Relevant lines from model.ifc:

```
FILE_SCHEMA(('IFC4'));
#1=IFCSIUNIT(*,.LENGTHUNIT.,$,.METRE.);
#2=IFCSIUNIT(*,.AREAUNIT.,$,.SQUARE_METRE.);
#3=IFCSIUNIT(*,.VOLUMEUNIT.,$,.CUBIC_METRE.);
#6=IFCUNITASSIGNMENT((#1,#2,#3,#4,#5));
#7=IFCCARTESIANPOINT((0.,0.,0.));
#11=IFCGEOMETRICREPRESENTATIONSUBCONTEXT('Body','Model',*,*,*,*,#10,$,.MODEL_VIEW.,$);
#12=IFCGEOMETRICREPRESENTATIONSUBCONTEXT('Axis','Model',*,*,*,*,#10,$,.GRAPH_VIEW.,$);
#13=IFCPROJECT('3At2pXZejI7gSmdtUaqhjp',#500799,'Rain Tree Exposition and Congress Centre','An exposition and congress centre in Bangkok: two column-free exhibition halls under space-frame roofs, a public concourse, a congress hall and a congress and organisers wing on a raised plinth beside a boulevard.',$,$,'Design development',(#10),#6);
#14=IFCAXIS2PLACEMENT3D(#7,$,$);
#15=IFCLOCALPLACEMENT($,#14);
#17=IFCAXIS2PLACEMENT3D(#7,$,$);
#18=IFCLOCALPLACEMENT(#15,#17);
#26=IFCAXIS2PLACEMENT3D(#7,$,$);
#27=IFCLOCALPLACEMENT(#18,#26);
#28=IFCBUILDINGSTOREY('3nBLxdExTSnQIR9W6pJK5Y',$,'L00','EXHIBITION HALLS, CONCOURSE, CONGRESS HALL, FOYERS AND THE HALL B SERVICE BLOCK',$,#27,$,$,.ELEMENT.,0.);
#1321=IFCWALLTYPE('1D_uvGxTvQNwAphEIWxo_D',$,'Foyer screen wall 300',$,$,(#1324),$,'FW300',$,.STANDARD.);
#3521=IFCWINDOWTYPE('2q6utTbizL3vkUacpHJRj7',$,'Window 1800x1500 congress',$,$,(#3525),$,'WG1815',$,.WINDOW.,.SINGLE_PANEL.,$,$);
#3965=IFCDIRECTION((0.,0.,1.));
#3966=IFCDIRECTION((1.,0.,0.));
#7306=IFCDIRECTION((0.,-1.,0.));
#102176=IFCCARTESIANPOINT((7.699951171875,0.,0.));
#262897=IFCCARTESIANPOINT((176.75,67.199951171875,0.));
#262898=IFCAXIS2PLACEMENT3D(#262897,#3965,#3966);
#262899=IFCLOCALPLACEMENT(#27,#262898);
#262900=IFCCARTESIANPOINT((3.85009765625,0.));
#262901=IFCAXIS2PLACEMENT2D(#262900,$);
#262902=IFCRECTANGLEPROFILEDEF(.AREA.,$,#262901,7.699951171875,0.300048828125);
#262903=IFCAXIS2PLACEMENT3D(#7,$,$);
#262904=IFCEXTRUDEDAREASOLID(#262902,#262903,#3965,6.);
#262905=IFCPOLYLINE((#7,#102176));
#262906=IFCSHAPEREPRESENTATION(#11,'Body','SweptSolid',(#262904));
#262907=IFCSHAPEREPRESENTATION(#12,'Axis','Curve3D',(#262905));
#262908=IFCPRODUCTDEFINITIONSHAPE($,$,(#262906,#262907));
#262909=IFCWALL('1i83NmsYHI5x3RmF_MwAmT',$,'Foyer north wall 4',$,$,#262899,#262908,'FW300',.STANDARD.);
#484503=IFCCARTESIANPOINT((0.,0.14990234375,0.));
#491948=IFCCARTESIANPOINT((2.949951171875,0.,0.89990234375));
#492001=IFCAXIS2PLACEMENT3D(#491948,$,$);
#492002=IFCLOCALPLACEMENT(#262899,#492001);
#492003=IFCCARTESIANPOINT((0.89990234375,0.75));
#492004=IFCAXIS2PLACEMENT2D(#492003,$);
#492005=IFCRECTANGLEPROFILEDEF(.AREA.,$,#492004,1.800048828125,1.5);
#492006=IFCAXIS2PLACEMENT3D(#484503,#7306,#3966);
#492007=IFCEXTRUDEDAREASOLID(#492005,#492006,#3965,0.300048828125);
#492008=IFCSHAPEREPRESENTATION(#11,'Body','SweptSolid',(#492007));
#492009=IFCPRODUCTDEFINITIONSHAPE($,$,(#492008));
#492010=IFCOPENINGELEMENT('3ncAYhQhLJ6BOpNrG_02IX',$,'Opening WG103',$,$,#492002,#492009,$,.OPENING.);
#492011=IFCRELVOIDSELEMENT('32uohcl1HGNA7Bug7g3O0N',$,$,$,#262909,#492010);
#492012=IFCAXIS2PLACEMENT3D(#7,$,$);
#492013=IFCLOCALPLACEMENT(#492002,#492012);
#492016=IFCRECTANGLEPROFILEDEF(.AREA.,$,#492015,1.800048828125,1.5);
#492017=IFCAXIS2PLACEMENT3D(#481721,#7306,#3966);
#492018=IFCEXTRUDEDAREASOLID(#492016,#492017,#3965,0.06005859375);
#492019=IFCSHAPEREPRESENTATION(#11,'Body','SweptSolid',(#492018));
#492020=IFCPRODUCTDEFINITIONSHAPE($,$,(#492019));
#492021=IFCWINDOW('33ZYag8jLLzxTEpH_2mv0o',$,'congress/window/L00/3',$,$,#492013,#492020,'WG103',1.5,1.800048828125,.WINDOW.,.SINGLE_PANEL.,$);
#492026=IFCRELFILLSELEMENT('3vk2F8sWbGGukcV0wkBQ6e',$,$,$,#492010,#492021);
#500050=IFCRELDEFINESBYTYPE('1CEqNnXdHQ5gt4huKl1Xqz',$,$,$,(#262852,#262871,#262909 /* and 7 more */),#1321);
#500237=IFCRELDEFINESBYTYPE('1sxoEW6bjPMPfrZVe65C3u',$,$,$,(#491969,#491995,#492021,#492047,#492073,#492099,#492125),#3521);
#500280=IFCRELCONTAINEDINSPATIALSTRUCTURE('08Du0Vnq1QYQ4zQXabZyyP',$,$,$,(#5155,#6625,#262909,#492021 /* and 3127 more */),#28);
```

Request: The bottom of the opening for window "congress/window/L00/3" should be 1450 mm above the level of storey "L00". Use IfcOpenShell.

```python
import numpy as np
import ifcopenshell
import ifcopenshell.api.geometry
import ifcopenshell.geom
import ifcopenshell.util.element
import ifcopenshell.util.placement
import ifcopenshell.util.shape
import ifcopenshell.util.unit

model = ifcopenshell.open("model.ifc")
unit_scale = ifcopenshell.util.unit.calculate_unit_scale(model)

window = model.by_guid("33ZYag8jLLzxTEpH_2mv0o")
opening = window.FillsVoids[0].RelatingOpeningElement
storey = ifcopenshell.util.element.get_container(window, ifc_class="IfcBuildingStorey")
level = ifcopenshell.util.placement.get_local_placement(storey.ObjectPlacement)[2, 3]

# The opening's origin need not be at the sill, so measure its lowest point.
shape = ifcopenshell.geom.create_shape(ifcopenshell.geom.settings(), opening)
bottom = ifcopenshell.util.shape.get_shape_bottom_elevation(shape, shape.geometry) / unit_scale
dz = level + 1.45 - bottom

shift = np.array([0.0, 0.0, dz])
# The window is placed relative to its opening, so it follows when the opening moves.
matrix = ifcopenshell.util.placement.get_local_placement(opening.ObjectPlacement)
matrix[:3, 3] += shift
ifcopenshell.api.geometry.edit_object_placement(
    model, product=opening, matrix=matrix, is_si=False, should_transform_children=True
)

print(f"moved by {dz * unit_scale:+.3f} m")

model.write("model_updated.ifc")
```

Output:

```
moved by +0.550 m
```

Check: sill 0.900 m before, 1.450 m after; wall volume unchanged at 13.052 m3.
